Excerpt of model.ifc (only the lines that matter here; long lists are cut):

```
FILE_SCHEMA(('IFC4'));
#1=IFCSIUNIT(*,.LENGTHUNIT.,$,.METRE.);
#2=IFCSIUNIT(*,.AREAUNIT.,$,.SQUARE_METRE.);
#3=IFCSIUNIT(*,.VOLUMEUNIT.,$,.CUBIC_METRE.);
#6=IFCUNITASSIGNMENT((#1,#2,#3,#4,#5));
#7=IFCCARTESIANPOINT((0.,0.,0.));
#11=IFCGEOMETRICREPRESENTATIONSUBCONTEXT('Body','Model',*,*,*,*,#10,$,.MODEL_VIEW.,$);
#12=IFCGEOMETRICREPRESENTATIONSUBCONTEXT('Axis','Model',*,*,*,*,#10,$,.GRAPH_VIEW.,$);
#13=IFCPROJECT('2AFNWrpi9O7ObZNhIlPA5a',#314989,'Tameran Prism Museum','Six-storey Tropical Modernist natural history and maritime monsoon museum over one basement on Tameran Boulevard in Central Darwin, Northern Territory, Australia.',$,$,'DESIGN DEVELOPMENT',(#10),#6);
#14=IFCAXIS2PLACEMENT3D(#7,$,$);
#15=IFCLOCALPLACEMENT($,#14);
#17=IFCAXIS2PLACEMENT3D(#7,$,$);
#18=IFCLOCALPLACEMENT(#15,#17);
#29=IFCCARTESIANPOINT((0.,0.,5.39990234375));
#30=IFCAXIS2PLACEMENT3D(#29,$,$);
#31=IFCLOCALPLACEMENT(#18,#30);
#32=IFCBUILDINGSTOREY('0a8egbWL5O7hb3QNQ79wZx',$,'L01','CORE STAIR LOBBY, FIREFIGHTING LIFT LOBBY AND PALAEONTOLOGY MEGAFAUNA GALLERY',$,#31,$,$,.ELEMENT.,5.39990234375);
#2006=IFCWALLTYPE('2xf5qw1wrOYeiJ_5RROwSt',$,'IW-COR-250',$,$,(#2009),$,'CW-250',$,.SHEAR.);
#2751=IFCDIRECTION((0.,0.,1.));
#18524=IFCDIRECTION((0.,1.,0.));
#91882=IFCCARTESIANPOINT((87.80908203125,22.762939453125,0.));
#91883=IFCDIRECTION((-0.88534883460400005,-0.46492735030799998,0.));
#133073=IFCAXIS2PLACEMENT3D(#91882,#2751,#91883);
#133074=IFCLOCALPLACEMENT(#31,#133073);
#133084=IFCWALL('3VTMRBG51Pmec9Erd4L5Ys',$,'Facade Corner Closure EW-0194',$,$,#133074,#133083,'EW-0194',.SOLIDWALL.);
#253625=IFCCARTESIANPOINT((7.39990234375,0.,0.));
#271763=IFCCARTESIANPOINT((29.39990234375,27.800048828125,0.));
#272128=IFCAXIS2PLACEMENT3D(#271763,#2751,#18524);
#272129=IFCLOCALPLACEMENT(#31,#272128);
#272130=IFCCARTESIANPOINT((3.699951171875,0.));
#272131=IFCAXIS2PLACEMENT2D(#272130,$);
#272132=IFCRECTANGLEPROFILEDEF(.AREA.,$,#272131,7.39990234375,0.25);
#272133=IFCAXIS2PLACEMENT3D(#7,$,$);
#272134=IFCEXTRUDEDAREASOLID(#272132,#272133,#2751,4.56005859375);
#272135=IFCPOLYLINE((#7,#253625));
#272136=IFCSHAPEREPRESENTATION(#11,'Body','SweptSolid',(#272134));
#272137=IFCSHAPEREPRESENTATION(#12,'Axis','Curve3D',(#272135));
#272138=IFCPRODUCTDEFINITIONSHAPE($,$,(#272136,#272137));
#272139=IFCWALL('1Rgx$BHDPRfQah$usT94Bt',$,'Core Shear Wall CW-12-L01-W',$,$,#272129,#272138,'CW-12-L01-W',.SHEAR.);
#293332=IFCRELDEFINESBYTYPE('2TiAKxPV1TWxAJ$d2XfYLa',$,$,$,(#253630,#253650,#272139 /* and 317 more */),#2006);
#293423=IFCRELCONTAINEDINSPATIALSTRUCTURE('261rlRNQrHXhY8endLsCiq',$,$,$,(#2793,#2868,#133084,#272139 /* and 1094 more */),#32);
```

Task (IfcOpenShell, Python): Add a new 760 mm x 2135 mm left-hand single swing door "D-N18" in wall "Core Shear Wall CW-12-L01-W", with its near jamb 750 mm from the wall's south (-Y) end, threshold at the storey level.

```python
import numpy as np
import ifcopenshell
import ifcopenshell.api.feature
import ifcopenshell.api.geometry
import ifcopenshell.api.root
import ifcopenshell.api.spatial
import ifcopenshell.geom
import ifcopenshell.util.element
import ifcopenshell.util.placement
import ifcopenshell.util.representation
import ifcopenshell.util.shape
import ifcopenshell.util.unit

model = ifcopenshell.open("model.ifc")
unit_scale = ifcopenshell.util.unit.calculate_unit_scale(model)
settings = ifcopenshell.geom.settings()


def volume(element):
    """Net volume in cubic metres, openings subtracted."""
    shape = ifcopenshell.geom.create_shape(settings, element)
    return ifcopenshell.util.shape.get_volume(shape.geometry)


wall = model.by_id(272139)
storey = ifcopenshell.util.element.get_container(wall, ifc_class="IfcBuildingStorey")
context = ifcopenshell.util.representation.get_context(model, "Model", "Body", "MODEL_VIEW")
before = volume(wall)

width, height, from_end, sill = 0.76, 2.135, 0.75, 0.0  # metres

# The wall runs along its own X axis, and the end named is its -X end.
wall_shape = ifcopenshell.geom.create_shape(settings, wall)
x, y, z = ifcopenshell.util.shape.get_vertices(wall_shape.geometry).T
start = x.min() + from_end
face, thickness = float(y.min()), float(y.max() - y.min())
wall_matrix = ifcopenshell.util.placement.get_local_placement(wall.ObjectPlacement)
level = ifcopenshell.util.placement.get_local_placement(storey.ObjectPlacement)[2, 3]


def in_wall(x, y):
    """Placement at x, y metres in the wall's axes, at sill height."""
    matrix = wall_matrix.copy()
    matrix[:, 3] = wall_matrix @ np.array([x / unit_scale, y / unit_scale, 0.0, 1.0])
    matrix[2, 3] = level + sill / unit_scale
    return matrix


# Opening: a box that overshoots both wall faces by 50 mm.
opening = ifcopenshell.api.root.create_entity(model, ifc_class="IfcOpeningElement", predefined_type="OPENING")
box = ifcopenshell.api.geometry.add_wall_representation(
    model, context=context, length=width, height=height, thickness=thickness + 0.1
)
ifcopenshell.api.geometry.assign_representation(model, product=opening, representation=box)
ifcopenshell.api.geometry.edit_object_placement(model, product=opening, matrix=in_wall(start, face - 0.05), is_si=False)
ifcopenshell.api.feature.add_feature(model, feature=opening, element=wall)

door = ifcopenshell.api.root.create_entity(model, ifc_class="IfcDoor", name="D-N18", predefined_type="DOOR")
door.OverallWidth, door.OverallHeight = width / unit_scale, height / unit_scale
door.OperationType = "SINGLE_SWING_LEFT"
body = ifcopenshell.api.geometry.add_door_representation(
    model,
    context=context,
    overall_width=door.OverallWidth,
    overall_height=door.OverallHeight,
    operation_type="SINGLE_SWING_LEFT",
    lining_properties={"LiningDepth": thickness / unit_scale, "ThresholdDepth": thickness / unit_scale},
)
ifcopenshell.api.geometry.assign_representation(model, product=door, representation=body)
ifcopenshell.api.spatial.assign_container(model, products=[door], relating_structure=storey)
ifcopenshell.api.feature.add_filling(model, opening=opening, element=door)

# The lining spans the wall, so the door starts at the wall face.
ifcopenshell.api.geometry.edit_object_placement(model, product=door, matrix=in_wall(start, face), is_si=False)

after = volume(wall)

print(f"wall volume {before:.3f} -> {after:.3f} m3")

model.write("model_updated.ifc")
```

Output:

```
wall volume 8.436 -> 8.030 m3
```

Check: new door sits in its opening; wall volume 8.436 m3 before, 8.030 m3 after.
